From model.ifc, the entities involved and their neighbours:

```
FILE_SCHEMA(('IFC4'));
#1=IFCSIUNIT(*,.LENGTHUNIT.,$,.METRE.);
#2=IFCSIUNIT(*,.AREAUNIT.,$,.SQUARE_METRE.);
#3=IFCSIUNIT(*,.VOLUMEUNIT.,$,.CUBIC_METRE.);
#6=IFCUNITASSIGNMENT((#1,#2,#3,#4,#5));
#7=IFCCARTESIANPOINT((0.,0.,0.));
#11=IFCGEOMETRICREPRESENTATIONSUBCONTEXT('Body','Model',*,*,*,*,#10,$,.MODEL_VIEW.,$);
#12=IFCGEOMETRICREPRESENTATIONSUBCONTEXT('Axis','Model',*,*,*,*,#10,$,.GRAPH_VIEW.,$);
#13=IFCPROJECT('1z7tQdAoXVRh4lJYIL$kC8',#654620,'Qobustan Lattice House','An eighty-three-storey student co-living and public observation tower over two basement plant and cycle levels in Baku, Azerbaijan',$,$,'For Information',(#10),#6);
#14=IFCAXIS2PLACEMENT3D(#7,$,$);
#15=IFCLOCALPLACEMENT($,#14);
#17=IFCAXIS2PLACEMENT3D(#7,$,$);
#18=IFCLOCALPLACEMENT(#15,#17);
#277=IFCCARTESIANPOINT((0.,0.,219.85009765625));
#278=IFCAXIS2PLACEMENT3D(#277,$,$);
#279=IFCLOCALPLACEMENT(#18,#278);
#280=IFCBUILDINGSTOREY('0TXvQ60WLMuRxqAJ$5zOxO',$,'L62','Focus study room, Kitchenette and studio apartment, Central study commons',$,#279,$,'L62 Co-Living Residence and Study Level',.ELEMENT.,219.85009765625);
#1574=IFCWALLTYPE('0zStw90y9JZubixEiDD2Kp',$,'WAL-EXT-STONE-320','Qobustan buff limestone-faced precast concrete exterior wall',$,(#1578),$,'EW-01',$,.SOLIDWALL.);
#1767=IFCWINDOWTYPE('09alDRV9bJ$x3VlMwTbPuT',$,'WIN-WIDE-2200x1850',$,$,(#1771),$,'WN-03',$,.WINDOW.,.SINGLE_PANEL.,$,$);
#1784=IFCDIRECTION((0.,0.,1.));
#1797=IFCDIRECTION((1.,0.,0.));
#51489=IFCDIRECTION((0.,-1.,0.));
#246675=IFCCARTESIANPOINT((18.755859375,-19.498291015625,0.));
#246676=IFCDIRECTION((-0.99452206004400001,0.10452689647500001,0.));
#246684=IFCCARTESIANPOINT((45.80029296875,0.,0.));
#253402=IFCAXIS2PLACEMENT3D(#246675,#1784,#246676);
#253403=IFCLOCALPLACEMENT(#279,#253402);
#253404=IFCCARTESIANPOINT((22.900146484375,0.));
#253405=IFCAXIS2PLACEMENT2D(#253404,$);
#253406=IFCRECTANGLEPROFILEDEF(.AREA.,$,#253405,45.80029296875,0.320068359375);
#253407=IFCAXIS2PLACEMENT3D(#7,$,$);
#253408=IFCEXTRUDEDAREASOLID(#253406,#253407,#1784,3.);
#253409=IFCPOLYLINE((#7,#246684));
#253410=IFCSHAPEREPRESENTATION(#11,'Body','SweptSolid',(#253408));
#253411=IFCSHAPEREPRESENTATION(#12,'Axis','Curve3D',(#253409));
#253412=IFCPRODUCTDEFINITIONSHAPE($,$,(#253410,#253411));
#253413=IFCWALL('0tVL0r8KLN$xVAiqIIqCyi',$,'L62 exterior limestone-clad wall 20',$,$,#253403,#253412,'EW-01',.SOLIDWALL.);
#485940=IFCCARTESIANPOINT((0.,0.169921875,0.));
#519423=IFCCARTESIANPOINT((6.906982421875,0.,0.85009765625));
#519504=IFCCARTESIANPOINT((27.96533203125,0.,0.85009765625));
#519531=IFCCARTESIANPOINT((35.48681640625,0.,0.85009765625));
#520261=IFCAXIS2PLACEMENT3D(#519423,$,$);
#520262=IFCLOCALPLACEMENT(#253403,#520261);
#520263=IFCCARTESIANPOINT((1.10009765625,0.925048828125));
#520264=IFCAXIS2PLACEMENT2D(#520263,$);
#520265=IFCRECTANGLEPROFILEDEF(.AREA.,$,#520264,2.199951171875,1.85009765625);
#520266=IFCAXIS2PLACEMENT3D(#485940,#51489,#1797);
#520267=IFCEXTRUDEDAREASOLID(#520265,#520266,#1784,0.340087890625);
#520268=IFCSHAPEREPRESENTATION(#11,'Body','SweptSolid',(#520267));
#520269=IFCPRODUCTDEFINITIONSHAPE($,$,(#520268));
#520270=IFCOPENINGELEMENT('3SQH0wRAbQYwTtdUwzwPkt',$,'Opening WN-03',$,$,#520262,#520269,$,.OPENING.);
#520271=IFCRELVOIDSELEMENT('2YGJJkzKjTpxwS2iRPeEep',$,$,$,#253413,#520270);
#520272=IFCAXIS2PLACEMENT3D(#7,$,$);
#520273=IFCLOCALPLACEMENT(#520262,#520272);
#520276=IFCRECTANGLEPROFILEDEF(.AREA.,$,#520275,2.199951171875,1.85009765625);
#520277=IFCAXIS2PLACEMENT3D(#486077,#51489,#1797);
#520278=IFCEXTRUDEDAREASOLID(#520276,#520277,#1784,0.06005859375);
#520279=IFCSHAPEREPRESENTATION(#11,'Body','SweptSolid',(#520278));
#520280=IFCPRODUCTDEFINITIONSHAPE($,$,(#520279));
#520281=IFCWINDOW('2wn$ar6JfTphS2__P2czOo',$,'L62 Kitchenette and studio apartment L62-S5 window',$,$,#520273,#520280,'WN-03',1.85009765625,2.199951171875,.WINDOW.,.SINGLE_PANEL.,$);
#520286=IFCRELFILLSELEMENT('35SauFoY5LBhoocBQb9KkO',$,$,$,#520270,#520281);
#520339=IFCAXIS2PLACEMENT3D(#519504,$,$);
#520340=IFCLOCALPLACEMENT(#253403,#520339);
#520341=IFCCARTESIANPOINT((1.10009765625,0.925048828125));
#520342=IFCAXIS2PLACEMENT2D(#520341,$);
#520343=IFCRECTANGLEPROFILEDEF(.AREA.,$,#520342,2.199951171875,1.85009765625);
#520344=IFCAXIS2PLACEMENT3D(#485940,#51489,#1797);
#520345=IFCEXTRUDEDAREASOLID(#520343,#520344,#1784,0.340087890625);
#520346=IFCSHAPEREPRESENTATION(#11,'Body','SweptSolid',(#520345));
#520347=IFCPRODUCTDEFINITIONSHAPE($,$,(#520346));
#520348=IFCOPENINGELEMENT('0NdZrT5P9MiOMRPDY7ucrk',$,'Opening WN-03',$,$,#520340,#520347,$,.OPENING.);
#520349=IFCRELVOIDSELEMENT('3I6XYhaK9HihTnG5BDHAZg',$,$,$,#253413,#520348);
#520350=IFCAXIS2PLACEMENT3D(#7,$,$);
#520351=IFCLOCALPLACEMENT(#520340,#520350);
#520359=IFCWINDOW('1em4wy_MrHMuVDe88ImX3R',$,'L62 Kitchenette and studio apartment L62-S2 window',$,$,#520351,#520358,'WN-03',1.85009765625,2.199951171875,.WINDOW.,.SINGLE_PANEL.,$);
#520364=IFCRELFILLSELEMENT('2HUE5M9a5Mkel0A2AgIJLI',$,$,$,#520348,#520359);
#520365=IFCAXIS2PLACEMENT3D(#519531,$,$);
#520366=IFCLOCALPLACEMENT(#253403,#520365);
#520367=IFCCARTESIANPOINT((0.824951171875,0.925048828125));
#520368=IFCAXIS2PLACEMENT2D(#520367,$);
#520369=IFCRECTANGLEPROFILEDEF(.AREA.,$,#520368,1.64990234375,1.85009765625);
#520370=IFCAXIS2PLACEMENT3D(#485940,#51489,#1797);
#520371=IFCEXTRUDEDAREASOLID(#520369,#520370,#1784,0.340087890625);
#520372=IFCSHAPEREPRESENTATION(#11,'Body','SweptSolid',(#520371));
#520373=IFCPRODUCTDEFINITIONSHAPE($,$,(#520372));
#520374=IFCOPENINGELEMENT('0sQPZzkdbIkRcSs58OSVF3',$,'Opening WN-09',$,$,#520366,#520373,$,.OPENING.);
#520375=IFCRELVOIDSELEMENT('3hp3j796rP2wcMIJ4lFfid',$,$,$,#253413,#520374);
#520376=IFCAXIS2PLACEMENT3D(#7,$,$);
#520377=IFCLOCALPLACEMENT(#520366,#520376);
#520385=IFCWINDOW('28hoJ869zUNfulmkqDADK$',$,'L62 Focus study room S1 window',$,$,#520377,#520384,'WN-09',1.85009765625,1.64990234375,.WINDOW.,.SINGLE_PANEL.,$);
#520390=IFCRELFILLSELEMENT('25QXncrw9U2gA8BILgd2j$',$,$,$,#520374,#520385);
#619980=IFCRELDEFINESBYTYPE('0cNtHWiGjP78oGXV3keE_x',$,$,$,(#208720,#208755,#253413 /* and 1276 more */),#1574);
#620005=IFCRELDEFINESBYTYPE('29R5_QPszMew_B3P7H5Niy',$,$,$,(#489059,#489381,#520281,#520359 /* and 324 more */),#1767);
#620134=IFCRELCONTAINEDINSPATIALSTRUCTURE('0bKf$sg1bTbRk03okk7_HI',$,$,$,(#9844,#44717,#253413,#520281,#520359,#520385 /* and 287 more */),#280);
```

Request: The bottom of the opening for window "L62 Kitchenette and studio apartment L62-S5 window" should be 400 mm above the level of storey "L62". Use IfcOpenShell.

```python
import numpy as np
import ifcopenshell
import ifcopenshell.api.geometry
import ifcopenshell.geom
import ifcopenshell.util.element
import ifcopenshell.util.placement
import ifcopenshell.util.shape
import ifcopenshell.util.unit

model = ifcopenshell.open("model.ifc")
unit_scale = ifcopenshell.util.unit.calculate_unit_scale(model)

window = model.by_id(520281)
opening = window.FillsVoids[0].RelatingOpeningElement
storey = ifcopenshell.util.element.get_container(window, ifc_class="IfcBuildingStorey")
level = ifcopenshell.util.placement.get_local_placement(storey.ObjectPlacement)[2, 3]

# The opening's origin need not be at the sill, so measure its lowest point.
shape = ifcopenshell.geom.create_shape(ifcopenshell.geom.settings(), opening)
bottom = ifcopenshell.util.shape.get_shape_bottom_elevation(shape, shape.geometry) / unit_scale
dz = level + 0.4 / unit_scale - bottom

shift = np.array([0.0, 0.0, dz])
# The window is placed relative to its opening, so it follows when the opening moves.
matrix = ifcopenshell.util.placement.get_local_placement(opening.ObjectPlacement)
matrix[:3, 3] += shift
ifcopenshell.api.geometry.edit_object_placement(
    model, product=opening, matrix=matrix, is_si=False, should_transform_children=True
)

print(f"moved by {dz * unit_scale:+.3f} m")

model.write("model-out.ifc")
```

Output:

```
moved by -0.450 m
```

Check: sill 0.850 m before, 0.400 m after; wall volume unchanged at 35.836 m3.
